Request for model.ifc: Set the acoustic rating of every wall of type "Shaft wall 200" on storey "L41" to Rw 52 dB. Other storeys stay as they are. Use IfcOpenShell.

First a look at what the model holds.

```python
import ifcopenshell
import ifcopenshell.util.element

model = ifcopenshell.open("model.ifc")
print(model.schema)
storey = next(s for s in model.by_type("IfcBuildingStorey") if s.Name == "L41")
walls = [e for e in ifcopenshell.util.element.get_decomposition(storey) if e.is_a("IfcWall")]
seen = {}
for e in walls:
    element_type = ifcopenshell.util.element.get_type(e)
    key = (element_type.Name if element_type != e and element_type else None, ifcopenshell.util.element.get_pset(e, "Pset_WallCommon", "AcousticRating"))
    seen[key] = seen.get(key, 0) + 1
for (name, value), count in sorted(seen.items(), key=str):
    print(count, "x", name, "|", value)
```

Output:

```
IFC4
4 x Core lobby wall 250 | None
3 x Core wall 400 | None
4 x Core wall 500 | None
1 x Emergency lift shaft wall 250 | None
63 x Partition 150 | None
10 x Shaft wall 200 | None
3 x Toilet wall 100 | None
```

```python
import ifcopenshell
import ifcopenshell.api.pset
import ifcopenshell.util.element

model = ifcopenshell.open("model.ifc")

storey = next(s for s in model.by_type("IfcBuildingStorey") if s.Name == "L41")
walls = [e for e in ifcopenshell.util.element.get_decomposition(storey) if e.is_a("IfcWall")]

count = 0
for e in walls:
    element_type = ifcopenshell.util.element.get_type(e)
    if element_type in (None, e) or element_type.Name != "Shaft wall 200":
        continue
    found = ifcopenshell.util.element.get_pset(e, "Pset_WallCommon", should_inherit=False)
    if found:
        pset = model.by_id(found["id"])
        if len(ifcopenshell.util.element.get_elements_by_pset(pset)) > 1:
            pset = ifcopenshell.api.pset.unshare_pset(model, products=[e], pset=pset)[0]
    else:
        pset = ifcopenshell.api.pset.add_pset(model, product=e, name="Pset_WallCommon")
    ifcopenshell.api.pset.edit_pset(model, pset=pset, properties={"AcousticRating": "Rw 52 dB"})
    count += 1

print(count, "walls updated")

model.write("model-out.ifc")
```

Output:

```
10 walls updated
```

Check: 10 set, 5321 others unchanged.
